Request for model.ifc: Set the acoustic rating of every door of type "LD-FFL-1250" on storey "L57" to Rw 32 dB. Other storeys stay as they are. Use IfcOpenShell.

First a look at what the model holds.

```python
import ifcopenshell
import ifcopenshell.util.element

model = ifcopenshell.open("model.ifc")
print(model.schema)
storey = next(s for s in model.by_type("IfcBuildingStorey") if s.Name == "L57")
doors = [e for e in ifcopenshell.util.element.get_decomposition(storey) if e.is_a("IfcDoor")]
seen = {}
for e in doors:
    element_type = ifcopenshell.util.element.get_type(e)
    key = (element_type.Name if element_type != e and element_type else None, ifcopenshell.util.element.get_pset(e, "Pset_DoorCommon", "AcousticRating"))
    seen[key] = seen.get(key, 0) + 1
for (name, value), count in sorted(seen.items(), key=str):
    print(count, "x", name, "|", value)
```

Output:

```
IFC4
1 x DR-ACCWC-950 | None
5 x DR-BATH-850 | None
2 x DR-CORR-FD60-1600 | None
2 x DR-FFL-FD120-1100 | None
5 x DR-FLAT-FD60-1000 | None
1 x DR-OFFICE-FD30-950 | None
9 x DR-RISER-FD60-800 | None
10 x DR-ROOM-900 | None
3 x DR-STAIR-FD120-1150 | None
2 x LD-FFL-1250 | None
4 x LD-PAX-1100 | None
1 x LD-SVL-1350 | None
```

```python
import ifcopenshell
import ifcopenshell.api.pset
import ifcopenshell.util.element

model = ifcopenshell.open("model.ifc")

storey = next(s for s in model.by_type("IfcBuildingStorey") if s.Name == "L57")
doors = [e for e in ifcopenshell.util.element.get_decomposition(storey) if e.is_a("IfcDoor")]

count = 0
for e in doors:
    element_type = ifcopenshell.util.element.get_type(e)
    if element_type in (None, e) or element_type.Name != "LD-FFL-1250":
        continue
    # add_pset returns the element's existing set when there is one.
    pset = ifcopenshell.api.pset.add_pset(model, product=e, name="Pset_DoorCommon")
    ifcopenshell.api.pset.edit_pset(model, pset=pset, properties={"AcousticRating": "Rw 32 dB"})
    count += 1

print(count, "doors updated")

model.write("model_v2.ifc")
```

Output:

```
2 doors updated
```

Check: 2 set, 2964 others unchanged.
